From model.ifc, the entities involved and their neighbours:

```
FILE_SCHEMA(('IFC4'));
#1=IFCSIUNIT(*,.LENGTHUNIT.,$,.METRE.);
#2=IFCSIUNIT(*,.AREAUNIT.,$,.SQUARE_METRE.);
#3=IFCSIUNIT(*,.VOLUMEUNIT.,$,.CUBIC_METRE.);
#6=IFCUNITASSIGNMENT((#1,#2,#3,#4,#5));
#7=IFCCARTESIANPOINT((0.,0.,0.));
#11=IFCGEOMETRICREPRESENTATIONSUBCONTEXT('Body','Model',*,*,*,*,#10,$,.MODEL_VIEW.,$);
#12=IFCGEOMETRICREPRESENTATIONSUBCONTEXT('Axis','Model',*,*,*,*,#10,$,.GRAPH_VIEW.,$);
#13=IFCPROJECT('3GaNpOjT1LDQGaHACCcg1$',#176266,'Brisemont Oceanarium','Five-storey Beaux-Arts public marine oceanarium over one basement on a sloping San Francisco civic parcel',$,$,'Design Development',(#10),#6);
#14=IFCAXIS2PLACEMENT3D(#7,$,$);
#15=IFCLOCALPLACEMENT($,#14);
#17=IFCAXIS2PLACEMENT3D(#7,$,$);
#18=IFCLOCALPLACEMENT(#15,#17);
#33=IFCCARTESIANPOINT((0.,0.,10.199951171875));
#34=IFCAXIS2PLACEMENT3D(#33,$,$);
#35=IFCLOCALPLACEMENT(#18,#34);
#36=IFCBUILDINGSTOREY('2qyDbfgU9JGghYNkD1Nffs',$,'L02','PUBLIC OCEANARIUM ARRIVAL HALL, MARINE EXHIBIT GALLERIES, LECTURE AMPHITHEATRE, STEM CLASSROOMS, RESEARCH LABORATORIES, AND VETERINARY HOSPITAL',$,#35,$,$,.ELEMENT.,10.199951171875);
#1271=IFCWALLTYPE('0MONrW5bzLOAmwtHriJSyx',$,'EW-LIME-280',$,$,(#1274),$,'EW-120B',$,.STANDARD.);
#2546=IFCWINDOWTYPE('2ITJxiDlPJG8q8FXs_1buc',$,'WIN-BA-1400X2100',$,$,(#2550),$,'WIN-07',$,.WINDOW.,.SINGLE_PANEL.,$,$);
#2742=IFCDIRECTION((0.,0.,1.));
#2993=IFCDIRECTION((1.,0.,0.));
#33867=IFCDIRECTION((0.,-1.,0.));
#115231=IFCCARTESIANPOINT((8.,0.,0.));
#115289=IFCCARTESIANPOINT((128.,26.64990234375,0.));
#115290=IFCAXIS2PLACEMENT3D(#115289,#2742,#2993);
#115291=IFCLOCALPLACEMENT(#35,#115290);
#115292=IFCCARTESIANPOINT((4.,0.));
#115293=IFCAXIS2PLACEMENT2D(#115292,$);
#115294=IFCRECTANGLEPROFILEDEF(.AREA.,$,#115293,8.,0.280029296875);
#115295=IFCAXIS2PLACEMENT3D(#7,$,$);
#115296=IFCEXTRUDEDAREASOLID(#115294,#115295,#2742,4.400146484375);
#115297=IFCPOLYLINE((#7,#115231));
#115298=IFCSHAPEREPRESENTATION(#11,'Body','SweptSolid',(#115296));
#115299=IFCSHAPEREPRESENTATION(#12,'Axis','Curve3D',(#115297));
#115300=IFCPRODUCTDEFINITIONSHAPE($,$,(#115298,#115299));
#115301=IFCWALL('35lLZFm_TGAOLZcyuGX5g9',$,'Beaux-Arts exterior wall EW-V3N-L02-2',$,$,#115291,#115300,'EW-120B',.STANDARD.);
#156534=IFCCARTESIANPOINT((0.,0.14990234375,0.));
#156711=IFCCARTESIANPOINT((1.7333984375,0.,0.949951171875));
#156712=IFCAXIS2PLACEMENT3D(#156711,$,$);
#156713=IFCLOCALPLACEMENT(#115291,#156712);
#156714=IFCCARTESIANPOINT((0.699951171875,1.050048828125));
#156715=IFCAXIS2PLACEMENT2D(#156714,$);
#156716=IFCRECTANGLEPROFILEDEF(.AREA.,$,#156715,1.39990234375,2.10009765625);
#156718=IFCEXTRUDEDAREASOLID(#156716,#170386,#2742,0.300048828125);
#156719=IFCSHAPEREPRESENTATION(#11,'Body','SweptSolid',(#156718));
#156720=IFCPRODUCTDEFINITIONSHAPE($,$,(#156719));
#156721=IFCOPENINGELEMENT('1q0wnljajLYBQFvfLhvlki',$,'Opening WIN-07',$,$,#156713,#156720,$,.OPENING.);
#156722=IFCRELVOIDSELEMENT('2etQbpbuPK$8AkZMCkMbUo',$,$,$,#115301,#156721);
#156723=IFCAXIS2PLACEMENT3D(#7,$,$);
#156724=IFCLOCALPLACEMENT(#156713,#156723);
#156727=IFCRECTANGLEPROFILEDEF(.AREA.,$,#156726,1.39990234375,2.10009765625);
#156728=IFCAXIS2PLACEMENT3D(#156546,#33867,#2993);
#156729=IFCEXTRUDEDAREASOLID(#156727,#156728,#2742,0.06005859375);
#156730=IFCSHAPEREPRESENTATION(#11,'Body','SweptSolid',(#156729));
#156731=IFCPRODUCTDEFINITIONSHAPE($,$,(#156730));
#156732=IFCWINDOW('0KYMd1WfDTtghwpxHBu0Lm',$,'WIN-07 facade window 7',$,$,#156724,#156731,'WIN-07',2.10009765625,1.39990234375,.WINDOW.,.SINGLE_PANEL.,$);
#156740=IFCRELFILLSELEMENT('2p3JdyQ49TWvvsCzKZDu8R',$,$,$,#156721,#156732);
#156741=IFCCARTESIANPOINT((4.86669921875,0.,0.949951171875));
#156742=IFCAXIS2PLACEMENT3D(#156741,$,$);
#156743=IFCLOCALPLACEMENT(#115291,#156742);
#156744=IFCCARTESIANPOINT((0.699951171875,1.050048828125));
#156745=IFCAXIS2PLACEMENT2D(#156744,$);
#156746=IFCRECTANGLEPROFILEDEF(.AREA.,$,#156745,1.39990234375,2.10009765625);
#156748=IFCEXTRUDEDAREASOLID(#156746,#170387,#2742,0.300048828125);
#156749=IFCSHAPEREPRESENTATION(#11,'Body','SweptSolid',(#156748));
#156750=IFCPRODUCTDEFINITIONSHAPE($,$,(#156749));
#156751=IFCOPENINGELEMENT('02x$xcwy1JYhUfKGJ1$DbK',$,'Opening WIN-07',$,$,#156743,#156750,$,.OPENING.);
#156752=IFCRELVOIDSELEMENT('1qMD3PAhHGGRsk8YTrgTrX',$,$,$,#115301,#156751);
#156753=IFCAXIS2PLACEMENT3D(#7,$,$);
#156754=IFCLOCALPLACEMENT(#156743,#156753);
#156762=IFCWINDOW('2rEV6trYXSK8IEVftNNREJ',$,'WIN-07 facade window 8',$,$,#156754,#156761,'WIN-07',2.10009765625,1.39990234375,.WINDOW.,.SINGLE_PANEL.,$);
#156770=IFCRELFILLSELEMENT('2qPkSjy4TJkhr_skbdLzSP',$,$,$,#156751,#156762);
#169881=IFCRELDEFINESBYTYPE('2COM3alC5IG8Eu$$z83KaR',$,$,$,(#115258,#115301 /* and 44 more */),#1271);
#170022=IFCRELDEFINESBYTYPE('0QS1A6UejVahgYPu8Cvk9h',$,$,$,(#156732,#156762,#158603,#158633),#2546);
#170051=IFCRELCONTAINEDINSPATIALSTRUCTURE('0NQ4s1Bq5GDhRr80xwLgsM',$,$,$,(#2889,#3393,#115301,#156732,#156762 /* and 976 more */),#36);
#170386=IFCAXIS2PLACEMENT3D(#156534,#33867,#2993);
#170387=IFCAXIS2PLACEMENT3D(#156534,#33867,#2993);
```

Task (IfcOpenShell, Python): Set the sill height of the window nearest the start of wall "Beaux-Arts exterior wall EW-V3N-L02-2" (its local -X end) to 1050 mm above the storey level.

```python
import numpy as np
import ifcopenshell
import ifcopenshell.api.geometry
import ifcopenshell.geom
import ifcopenshell.util.element
import ifcopenshell.util.placement
import ifcopenshell.util.shape
import ifcopenshell.util.unit

model = ifcopenshell.open("model.ifc")
unit_scale = ifcopenshell.util.unit.calculate_unit_scale(model)

window = model.by_guid("0KYMd1WfDTtghwpxHBu0Lm")
opening = window.FillsVoids[0].RelatingOpeningElement
storey = ifcopenshell.util.element.get_container(window, ifc_class="IfcBuildingStorey")
level = ifcopenshell.util.placement.get_local_placement(storey.ObjectPlacement)[2, 3]

# The opening's origin need not be at the sill, so measure its lowest point.
shape = ifcopenshell.geom.create_shape(ifcopenshell.geom.settings(), opening)
bottom = ifcopenshell.util.shape.get_shape_bottom_elevation(shape, shape.geometry) / unit_scale
dz = level + 1.05 / unit_scale - bottom

shift = np.array([0.0, 0.0, dz])
# The window is placed relative to its opening, so it follows when the opening moves.
matrix = ifcopenshell.util.placement.get_local_placement(opening.ObjectPlacement)
matrix[:3, 3] += shift
ifcopenshell.api.geometry.edit_object_placement(
    model, product=opening, matrix=matrix, is_si=False, should_transform_children=True
)

print(f"moved by {dz * unit_scale:+.3f} m")

model.write("model-out.ifc")
```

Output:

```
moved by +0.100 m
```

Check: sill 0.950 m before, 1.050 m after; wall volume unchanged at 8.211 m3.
